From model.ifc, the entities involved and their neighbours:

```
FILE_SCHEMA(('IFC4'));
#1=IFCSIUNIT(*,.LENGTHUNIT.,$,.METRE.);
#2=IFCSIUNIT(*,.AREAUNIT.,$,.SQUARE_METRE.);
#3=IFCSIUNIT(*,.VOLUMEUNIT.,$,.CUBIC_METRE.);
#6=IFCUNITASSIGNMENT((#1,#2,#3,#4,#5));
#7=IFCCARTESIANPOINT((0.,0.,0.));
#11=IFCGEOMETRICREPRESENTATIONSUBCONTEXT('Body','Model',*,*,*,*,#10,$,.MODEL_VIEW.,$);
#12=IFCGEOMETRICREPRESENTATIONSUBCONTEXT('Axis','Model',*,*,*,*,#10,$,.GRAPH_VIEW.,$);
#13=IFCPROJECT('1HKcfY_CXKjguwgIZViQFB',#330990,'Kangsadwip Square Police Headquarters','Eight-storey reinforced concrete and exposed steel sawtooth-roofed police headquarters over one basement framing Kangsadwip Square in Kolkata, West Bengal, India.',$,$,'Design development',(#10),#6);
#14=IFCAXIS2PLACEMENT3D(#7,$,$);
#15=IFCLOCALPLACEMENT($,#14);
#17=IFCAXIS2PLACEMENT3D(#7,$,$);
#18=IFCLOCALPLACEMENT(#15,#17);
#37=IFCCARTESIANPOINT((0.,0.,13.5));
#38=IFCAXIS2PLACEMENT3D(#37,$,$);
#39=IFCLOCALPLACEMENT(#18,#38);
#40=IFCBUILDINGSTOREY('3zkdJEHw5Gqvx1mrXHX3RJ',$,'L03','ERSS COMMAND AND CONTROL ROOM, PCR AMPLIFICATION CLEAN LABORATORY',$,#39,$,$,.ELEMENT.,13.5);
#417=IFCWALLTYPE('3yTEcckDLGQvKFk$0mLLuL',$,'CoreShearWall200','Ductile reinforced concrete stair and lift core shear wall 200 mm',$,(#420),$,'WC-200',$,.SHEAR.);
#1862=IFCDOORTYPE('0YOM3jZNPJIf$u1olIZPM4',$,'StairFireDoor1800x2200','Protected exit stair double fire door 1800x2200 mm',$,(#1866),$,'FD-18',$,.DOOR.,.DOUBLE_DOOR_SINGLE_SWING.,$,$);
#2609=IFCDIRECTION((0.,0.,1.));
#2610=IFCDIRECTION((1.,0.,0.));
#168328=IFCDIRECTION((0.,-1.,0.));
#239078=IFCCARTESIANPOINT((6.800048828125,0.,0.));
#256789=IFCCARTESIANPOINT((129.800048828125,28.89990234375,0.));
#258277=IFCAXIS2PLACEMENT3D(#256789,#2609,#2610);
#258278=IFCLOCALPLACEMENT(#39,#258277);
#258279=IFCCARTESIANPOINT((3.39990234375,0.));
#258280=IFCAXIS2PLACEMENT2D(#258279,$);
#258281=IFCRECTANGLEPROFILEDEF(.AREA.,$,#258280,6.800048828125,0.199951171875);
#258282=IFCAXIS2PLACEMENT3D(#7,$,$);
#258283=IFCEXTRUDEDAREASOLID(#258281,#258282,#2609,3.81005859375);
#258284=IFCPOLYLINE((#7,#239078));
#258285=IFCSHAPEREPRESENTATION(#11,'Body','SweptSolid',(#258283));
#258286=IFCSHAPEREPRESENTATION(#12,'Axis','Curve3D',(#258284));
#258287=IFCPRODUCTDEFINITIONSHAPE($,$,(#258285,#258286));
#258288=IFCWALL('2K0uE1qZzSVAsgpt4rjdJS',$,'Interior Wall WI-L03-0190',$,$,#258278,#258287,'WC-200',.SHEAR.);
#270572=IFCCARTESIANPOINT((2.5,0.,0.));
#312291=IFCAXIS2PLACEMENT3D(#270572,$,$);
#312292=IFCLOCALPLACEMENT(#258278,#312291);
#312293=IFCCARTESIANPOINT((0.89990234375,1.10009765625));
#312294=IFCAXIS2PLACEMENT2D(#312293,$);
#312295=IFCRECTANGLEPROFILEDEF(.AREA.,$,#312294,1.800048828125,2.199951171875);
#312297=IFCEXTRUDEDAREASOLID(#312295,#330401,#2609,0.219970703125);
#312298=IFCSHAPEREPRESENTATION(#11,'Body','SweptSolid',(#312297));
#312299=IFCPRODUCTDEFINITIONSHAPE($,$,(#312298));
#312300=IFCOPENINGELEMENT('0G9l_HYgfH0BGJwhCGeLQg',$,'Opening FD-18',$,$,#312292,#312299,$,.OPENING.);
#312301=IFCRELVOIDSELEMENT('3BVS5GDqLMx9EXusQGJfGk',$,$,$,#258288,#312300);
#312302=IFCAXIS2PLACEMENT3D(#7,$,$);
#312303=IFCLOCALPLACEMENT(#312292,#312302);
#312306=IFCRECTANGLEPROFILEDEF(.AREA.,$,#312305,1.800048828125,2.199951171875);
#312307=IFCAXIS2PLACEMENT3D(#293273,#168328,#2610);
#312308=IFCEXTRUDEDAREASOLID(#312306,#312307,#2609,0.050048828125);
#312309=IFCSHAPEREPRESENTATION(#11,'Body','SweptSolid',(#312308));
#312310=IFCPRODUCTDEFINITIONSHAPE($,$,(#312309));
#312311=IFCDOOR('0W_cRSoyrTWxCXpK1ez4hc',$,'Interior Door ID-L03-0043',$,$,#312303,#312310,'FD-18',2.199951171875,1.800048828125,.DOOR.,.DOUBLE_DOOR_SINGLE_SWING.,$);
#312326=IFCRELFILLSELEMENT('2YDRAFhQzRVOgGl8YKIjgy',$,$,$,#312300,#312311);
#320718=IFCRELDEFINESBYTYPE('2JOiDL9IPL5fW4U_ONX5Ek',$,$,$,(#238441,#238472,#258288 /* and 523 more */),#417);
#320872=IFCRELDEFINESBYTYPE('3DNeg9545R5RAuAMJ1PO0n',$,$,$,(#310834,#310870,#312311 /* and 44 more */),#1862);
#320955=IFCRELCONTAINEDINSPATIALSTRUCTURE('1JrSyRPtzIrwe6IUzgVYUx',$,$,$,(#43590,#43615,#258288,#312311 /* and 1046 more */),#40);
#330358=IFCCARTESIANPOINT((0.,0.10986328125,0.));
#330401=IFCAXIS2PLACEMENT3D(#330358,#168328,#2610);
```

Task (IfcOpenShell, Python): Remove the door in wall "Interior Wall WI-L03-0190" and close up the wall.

```python
import ifcopenshell
import ifcopenshell.api.feature
import ifcopenshell.api.root
import ifcopenshell.geom
import ifcopenshell.util.shape

model = ifcopenshell.open("model.ifc")
settings = ifcopenshell.geom.settings()


def volume(element):
    """Net volume in cubic metres, openings subtracted."""
    shape = ifcopenshell.geom.create_shape(settings, element)
    return ifcopenshell.util.shape.get_volume(shape.geometry)


door = model.by_guid("0W_cRSoyrTWxCXpK1ez4hc")
opening = door.FillsVoids[0].RelatingOpeningElement
wall = opening.VoidsElements[0].RelatingBuildingElement
before = volume(wall)

ifcopenshell.api.root.remove_product(model, product=door)
ifcopenshell.api.feature.remove_feature(model, feature=opening)

after = volume(wall)

print(f"wall volume {before:.3f} -> {after:.3f} m3")

model.write("model_updated.ifc")
```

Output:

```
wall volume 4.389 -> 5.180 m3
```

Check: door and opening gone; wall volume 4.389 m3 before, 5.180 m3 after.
